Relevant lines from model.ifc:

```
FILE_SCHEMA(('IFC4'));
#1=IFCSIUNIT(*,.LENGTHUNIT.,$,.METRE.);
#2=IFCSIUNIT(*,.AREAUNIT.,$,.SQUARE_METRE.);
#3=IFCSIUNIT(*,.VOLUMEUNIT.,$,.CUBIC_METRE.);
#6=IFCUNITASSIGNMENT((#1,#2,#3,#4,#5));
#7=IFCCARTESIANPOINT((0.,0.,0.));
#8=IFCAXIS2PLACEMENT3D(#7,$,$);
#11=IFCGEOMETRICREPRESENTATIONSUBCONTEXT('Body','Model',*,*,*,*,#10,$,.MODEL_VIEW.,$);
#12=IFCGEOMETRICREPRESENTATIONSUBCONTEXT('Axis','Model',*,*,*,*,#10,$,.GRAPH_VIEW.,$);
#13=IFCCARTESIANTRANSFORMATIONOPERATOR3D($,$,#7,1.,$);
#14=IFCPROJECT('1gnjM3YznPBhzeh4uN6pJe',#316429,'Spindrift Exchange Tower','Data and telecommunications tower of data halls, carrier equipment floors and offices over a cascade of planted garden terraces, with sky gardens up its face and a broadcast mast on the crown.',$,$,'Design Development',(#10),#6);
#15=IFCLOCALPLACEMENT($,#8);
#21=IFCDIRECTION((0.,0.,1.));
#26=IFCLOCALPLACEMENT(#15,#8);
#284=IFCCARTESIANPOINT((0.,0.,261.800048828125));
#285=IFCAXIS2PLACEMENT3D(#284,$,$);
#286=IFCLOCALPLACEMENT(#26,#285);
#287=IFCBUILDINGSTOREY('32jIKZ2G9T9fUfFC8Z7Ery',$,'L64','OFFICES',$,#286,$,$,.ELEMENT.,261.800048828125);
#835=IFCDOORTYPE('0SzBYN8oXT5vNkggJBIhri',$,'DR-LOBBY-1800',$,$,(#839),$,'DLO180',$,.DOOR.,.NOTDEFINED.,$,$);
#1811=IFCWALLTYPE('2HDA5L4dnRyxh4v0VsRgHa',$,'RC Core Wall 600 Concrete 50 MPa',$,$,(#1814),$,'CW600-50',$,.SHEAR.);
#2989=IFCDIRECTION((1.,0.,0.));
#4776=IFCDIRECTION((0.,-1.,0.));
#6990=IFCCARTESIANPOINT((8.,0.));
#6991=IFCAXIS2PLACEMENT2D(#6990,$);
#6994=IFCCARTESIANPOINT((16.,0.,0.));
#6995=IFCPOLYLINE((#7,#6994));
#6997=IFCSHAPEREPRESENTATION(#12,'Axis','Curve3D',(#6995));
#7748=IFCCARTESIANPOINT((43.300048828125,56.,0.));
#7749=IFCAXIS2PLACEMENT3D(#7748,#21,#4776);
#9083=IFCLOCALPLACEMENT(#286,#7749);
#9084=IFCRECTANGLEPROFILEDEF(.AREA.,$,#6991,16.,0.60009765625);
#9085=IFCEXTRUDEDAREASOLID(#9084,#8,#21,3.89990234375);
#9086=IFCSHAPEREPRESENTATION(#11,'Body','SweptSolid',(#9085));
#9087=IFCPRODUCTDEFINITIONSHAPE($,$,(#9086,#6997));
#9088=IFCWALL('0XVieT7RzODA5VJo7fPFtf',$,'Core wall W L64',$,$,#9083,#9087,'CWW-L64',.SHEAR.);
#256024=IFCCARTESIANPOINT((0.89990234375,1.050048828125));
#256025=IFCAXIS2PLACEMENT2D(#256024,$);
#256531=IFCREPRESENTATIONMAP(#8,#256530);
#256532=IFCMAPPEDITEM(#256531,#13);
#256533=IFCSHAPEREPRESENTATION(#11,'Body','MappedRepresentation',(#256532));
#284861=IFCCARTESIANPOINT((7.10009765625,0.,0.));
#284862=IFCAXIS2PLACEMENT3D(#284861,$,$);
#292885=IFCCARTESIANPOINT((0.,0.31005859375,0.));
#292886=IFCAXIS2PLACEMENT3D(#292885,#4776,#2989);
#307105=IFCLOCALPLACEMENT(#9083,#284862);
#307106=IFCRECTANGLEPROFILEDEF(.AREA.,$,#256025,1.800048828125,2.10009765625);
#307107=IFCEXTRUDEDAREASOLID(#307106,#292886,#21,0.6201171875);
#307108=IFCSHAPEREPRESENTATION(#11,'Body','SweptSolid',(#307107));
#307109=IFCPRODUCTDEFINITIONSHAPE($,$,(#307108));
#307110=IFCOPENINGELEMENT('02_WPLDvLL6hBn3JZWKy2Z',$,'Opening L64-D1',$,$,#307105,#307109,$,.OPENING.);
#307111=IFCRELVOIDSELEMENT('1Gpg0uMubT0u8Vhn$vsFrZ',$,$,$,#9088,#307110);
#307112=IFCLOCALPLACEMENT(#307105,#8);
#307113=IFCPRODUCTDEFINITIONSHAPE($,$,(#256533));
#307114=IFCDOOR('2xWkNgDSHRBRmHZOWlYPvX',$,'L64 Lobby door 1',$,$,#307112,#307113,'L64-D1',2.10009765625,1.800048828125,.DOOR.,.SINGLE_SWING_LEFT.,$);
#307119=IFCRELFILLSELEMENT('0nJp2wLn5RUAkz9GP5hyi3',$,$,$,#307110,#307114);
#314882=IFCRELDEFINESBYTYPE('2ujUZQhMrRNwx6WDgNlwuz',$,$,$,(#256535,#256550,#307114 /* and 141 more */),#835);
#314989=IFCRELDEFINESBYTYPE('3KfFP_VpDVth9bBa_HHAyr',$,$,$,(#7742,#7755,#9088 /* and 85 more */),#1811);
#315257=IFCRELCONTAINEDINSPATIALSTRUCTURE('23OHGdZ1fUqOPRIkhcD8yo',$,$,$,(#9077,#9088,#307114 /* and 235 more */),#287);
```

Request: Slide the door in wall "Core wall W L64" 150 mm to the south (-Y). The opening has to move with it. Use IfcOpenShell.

```python
import ifcopenshell
import ifcopenshell.api.geometry
import ifcopenshell.util.placement

model = ifcopenshell.open("model.ifc")

door = model.by_guid("2xWkNgDSHRBRmHZOWlYPvX")
opening = door.FillsVoids[0].RelatingOpeningElement
wall = opening.VoidsElements[0].RelatingBuildingElement

wall_matrix = ifcopenshell.util.placement.get_local_placement(wall.ObjectPlacement)
shift = wall_matrix[:3, 0] * 0.15
before = ifcopenshell.util.placement.get_local_placement(door.ObjectPlacement)[:3, 3].copy()

# The door is placed relative to its opening, so it follows when the opening moves.
matrix = ifcopenshell.util.placement.get_local_placement(opening.ObjectPlacement)
matrix[:3, 3] += shift
ifcopenshell.api.geometry.edit_object_placement(
    model, product=opening, matrix=matrix, is_si=False, should_transform_children=True
)

after = ifcopenshell.util.placement.get_local_placement(door.ObjectPlacement)[:3, 3]
print("door moved by", (after - before).round(3) + 0.0)

model.write("model-out.ifc")
```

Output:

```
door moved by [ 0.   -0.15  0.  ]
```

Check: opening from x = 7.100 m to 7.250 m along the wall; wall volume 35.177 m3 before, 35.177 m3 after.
